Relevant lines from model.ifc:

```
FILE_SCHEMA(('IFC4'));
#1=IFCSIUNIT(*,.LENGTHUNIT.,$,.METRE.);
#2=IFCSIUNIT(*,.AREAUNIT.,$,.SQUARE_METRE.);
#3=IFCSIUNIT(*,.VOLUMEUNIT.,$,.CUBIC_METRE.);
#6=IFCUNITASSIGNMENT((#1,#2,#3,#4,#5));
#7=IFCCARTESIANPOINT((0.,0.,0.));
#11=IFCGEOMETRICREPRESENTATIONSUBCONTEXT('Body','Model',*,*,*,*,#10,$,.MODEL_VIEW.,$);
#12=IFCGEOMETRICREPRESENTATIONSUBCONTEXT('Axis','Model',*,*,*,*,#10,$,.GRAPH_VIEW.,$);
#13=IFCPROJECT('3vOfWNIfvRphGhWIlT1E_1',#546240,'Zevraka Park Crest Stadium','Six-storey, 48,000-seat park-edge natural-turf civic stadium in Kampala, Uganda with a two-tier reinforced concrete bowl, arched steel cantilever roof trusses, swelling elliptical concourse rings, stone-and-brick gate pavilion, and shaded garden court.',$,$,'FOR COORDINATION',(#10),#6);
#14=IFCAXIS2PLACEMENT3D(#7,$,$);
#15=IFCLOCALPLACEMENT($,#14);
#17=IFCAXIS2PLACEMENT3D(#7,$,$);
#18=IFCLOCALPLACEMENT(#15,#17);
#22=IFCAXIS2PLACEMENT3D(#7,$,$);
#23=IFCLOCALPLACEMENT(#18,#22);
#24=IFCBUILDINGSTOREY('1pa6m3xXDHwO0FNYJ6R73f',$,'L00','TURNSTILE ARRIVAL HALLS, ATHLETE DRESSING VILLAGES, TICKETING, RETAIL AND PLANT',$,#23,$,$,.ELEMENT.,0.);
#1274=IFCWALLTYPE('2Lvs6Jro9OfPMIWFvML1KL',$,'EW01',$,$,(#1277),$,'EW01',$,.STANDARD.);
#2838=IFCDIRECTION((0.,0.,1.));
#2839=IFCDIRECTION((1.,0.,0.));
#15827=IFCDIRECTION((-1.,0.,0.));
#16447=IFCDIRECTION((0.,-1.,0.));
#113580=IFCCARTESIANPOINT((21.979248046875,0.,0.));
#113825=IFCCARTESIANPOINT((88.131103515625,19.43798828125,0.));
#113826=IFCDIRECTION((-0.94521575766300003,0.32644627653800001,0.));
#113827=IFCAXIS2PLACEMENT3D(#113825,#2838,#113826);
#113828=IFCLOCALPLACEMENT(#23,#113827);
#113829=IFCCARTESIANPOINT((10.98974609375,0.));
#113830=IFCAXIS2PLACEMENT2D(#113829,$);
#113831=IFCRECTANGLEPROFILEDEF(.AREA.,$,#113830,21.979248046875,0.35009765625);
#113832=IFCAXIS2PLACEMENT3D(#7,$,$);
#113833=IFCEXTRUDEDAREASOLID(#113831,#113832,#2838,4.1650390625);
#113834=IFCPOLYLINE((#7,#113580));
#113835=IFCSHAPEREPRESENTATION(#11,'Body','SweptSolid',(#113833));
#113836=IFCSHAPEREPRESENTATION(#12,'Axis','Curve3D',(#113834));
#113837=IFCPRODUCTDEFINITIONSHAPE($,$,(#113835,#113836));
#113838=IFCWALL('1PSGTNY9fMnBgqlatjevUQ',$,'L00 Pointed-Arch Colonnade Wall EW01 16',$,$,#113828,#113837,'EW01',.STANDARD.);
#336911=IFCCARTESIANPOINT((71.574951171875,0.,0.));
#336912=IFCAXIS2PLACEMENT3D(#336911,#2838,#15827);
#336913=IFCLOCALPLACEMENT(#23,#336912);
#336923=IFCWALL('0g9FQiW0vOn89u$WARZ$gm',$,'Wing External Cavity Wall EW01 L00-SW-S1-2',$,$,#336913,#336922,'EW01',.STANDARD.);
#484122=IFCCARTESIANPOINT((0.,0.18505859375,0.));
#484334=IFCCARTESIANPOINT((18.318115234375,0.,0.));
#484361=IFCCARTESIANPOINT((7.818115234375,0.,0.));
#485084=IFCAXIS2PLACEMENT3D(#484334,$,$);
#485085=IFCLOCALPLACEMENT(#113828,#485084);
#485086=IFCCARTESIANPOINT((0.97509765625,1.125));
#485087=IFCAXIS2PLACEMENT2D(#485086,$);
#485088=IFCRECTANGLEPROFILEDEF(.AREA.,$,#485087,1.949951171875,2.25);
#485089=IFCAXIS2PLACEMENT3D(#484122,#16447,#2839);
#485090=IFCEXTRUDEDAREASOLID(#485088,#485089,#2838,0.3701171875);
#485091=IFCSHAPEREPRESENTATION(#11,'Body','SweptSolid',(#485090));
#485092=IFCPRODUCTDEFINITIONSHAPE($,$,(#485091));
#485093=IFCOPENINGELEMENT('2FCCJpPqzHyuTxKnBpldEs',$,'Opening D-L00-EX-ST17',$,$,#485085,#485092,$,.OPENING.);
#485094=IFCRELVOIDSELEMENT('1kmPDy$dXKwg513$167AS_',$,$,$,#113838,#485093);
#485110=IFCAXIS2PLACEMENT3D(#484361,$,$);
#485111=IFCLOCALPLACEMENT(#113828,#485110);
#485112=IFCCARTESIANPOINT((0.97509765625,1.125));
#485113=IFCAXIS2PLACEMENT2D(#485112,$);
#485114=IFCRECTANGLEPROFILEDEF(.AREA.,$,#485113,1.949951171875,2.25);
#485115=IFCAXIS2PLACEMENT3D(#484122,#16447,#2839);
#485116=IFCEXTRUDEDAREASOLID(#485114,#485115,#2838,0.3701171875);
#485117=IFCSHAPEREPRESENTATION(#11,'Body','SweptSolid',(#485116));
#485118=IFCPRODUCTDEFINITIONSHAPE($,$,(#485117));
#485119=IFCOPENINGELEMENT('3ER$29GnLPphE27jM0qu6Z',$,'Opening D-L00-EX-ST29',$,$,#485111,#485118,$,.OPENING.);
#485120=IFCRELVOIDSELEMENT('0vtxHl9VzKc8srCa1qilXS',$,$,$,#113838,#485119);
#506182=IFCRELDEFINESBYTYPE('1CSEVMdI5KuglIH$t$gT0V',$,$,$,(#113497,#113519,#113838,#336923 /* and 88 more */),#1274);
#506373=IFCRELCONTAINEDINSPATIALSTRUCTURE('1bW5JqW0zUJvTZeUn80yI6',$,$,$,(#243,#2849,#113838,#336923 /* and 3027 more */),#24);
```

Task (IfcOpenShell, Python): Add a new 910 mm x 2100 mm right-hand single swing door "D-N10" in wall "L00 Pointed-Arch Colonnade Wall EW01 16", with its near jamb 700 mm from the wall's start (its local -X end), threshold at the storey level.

```python
import numpy as np
import ifcopenshell
import ifcopenshell.api.feature
import ifcopenshell.api.geometry
import ifcopenshell.api.root
import ifcopenshell.api.spatial
import ifcopenshell.geom
import ifcopenshell.util.element
import ifcopenshell.util.placement
import ifcopenshell.util.representation
import ifcopenshell.util.shape
import ifcopenshell.util.unit

model = ifcopenshell.open("model.ifc")
unit_scale = ifcopenshell.util.unit.calculate_unit_scale(model)
settings = ifcopenshell.geom.settings()


def volume(element):
    """Net volume in cubic metres, openings subtracted."""
    shape = ifcopenshell.geom.create_shape(settings, element)
    return ifcopenshell.util.shape.get_volume(shape.geometry)


wall = model.by_guid("1PSGTNY9fMnBgqlatjevUQ")
storey = ifcopenshell.util.element.get_container(wall, ifc_class="IfcBuildingStorey")
context = ifcopenshell.util.representation.get_context(model, "Model", "Body", "MODEL_VIEW")
before = volume(wall)

width, height, from_end, sill = 0.91, 2.1, 0.7, 0.0  # metres

# The wall runs along its own X axis, and the end named is its -X end.
wall_shape = ifcopenshell.geom.create_shape(settings, wall)
x, y, z = ifcopenshell.util.shape.get_vertices(wall_shape.geometry).T
start = x.min() + from_end
face, thickness = float(y.min()), float(y.max() - y.min())
wall_matrix = ifcopenshell.util.placement.get_local_placement(wall.ObjectPlacement)
level = ifcopenshell.util.placement.get_local_placement(storey.ObjectPlacement)[2, 3]


def in_wall(x, y):
    """Placement at x, y metres in the wall's axes, at sill height."""
    matrix = wall_matrix.copy()
    matrix[:, 3] = wall_matrix @ np.array([x / unit_scale, y / unit_scale, 0.0, 1.0])
    matrix[2, 3] = level + sill / unit_scale
    return matrix


# Opening: a box that overshoots both wall faces by 50 mm.
opening = ifcopenshell.api.root.create_entity(model, ifc_class="IfcOpeningElement", predefined_type="OPENING")
box = ifcopenshell.api.geometry.add_wall_representation(
    model, context=context, length=width, height=height, thickness=thickness + 0.1
)
ifcopenshell.api.geometry.assign_representation(model, product=opening, representation=box)
ifcopenshell.api.geometry.edit_object_placement(model, product=opening, matrix=in_wall(start, face - 0.05), is_si=False)
ifcopenshell.api.feature.add_feature(model, feature=opening, element=wall)

door = ifcopenshell.api.root.create_entity(model, ifc_class="IfcDoor", name="D-N10", predefined_type="DOOR")
door.OverallWidth, door.OverallHeight = width / unit_scale, height / unit_scale
door.OperationType = "SINGLE_SWING_RIGHT"
body = ifcopenshell.api.geometry.add_door_representation(
    model,
    context=context,
    overall_width=door.OverallWidth,
    overall_height=door.OverallHeight,
    operation_type="SINGLE_SWING_RIGHT",
    lining_properties={"LiningDepth": thickness / unit_scale, "ThresholdDepth": thickness / unit_scale},
)
ifcopenshell.api.geometry.assign_representation(model, product=door, representation=body)
ifcopenshell.api.spatial.assign_container(model, products=[door], relating_structure=storey)
ifcopenshell.api.feature.add_filling(model, opening=opening, element=door)

# The lining spans the wall, so the door starts at the wall face.
ifcopenshell.api.geometry.edit_object_placement(model, product=door, matrix=in_wall(start, face), is_si=False)

after = volume(wall)

print(f"wall volume {before:.3f} -> {after:.3f} m3")

model.write("model_edited.ifc")
```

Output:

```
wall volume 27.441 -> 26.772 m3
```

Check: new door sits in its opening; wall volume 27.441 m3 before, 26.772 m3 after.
